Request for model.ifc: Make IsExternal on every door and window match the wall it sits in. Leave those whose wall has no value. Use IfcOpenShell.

First a look at what the model holds.

```python
import ifcopenshell
import ifcopenshell.util.element

model = ifcopenshell.open("model.ifc")
print(model.schema)
seen = {}
for e in model.by_type("IfcDoor") + model.by_type("IfcWindow"):
    if not e.FillsVoids:
        continue
    host = e.FillsVoids[0].RelatingOpeningElement.VoidsElements[0].RelatingBuildingElement
    own = ifcopenshell.util.element.get_pset(e, f"Pset_{e.is_a()[3:].removesuffix('StandardCase')}Common", "IsExternal")
    wall = ifcopenshell.util.element.get_pset(host, "Pset_WallCommon", "IsExternal")
    seen[e.is_a(), own, wall] = seen.get((e.is_a(), own, wall), 0) + 1
for (cls, own, wall), count in sorted(seen.items(), key=str):
    print(count, cls, "IsExternal:", own, "| host wall:", wall)
```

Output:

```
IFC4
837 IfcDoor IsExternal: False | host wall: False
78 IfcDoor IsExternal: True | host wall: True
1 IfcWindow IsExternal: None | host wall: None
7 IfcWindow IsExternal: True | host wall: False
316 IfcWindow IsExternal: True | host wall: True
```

```python
import ifcopenshell
import ifcopenshell.api.pset
import ifcopenshell.util.element

model = ifcopenshell.open("model.ifc")

count = 0
for ifc_class, pset_name in (("IfcDoor", "Pset_DoorCommon"), ("IfcWindow", "Pset_WindowCommon")):
    for e in model.by_type(ifc_class):
        if not e.FillsVoids:
            continue
        host = e.FillsVoids[0].RelatingOpeningElement.VoidsElements[0].RelatingBuildingElement
        external = ifcopenshell.util.element.get_pset(host, "Pset_WallCommon", "IsExternal")
        if external is None or ifcopenshell.util.element.get_pset(e, pset_name, "IsExternal") == external:
            continue
        pset = ifcopenshell.api.pset.add_pset(model, product=e, name=pset_name)
        ifcopenshell.api.pset.edit_pset(model, pset=pset, properties={"IsExternal": external})
        count += 1

print(count, "updated")

model.write("model_edited.ifc")
```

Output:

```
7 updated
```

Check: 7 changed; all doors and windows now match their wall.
